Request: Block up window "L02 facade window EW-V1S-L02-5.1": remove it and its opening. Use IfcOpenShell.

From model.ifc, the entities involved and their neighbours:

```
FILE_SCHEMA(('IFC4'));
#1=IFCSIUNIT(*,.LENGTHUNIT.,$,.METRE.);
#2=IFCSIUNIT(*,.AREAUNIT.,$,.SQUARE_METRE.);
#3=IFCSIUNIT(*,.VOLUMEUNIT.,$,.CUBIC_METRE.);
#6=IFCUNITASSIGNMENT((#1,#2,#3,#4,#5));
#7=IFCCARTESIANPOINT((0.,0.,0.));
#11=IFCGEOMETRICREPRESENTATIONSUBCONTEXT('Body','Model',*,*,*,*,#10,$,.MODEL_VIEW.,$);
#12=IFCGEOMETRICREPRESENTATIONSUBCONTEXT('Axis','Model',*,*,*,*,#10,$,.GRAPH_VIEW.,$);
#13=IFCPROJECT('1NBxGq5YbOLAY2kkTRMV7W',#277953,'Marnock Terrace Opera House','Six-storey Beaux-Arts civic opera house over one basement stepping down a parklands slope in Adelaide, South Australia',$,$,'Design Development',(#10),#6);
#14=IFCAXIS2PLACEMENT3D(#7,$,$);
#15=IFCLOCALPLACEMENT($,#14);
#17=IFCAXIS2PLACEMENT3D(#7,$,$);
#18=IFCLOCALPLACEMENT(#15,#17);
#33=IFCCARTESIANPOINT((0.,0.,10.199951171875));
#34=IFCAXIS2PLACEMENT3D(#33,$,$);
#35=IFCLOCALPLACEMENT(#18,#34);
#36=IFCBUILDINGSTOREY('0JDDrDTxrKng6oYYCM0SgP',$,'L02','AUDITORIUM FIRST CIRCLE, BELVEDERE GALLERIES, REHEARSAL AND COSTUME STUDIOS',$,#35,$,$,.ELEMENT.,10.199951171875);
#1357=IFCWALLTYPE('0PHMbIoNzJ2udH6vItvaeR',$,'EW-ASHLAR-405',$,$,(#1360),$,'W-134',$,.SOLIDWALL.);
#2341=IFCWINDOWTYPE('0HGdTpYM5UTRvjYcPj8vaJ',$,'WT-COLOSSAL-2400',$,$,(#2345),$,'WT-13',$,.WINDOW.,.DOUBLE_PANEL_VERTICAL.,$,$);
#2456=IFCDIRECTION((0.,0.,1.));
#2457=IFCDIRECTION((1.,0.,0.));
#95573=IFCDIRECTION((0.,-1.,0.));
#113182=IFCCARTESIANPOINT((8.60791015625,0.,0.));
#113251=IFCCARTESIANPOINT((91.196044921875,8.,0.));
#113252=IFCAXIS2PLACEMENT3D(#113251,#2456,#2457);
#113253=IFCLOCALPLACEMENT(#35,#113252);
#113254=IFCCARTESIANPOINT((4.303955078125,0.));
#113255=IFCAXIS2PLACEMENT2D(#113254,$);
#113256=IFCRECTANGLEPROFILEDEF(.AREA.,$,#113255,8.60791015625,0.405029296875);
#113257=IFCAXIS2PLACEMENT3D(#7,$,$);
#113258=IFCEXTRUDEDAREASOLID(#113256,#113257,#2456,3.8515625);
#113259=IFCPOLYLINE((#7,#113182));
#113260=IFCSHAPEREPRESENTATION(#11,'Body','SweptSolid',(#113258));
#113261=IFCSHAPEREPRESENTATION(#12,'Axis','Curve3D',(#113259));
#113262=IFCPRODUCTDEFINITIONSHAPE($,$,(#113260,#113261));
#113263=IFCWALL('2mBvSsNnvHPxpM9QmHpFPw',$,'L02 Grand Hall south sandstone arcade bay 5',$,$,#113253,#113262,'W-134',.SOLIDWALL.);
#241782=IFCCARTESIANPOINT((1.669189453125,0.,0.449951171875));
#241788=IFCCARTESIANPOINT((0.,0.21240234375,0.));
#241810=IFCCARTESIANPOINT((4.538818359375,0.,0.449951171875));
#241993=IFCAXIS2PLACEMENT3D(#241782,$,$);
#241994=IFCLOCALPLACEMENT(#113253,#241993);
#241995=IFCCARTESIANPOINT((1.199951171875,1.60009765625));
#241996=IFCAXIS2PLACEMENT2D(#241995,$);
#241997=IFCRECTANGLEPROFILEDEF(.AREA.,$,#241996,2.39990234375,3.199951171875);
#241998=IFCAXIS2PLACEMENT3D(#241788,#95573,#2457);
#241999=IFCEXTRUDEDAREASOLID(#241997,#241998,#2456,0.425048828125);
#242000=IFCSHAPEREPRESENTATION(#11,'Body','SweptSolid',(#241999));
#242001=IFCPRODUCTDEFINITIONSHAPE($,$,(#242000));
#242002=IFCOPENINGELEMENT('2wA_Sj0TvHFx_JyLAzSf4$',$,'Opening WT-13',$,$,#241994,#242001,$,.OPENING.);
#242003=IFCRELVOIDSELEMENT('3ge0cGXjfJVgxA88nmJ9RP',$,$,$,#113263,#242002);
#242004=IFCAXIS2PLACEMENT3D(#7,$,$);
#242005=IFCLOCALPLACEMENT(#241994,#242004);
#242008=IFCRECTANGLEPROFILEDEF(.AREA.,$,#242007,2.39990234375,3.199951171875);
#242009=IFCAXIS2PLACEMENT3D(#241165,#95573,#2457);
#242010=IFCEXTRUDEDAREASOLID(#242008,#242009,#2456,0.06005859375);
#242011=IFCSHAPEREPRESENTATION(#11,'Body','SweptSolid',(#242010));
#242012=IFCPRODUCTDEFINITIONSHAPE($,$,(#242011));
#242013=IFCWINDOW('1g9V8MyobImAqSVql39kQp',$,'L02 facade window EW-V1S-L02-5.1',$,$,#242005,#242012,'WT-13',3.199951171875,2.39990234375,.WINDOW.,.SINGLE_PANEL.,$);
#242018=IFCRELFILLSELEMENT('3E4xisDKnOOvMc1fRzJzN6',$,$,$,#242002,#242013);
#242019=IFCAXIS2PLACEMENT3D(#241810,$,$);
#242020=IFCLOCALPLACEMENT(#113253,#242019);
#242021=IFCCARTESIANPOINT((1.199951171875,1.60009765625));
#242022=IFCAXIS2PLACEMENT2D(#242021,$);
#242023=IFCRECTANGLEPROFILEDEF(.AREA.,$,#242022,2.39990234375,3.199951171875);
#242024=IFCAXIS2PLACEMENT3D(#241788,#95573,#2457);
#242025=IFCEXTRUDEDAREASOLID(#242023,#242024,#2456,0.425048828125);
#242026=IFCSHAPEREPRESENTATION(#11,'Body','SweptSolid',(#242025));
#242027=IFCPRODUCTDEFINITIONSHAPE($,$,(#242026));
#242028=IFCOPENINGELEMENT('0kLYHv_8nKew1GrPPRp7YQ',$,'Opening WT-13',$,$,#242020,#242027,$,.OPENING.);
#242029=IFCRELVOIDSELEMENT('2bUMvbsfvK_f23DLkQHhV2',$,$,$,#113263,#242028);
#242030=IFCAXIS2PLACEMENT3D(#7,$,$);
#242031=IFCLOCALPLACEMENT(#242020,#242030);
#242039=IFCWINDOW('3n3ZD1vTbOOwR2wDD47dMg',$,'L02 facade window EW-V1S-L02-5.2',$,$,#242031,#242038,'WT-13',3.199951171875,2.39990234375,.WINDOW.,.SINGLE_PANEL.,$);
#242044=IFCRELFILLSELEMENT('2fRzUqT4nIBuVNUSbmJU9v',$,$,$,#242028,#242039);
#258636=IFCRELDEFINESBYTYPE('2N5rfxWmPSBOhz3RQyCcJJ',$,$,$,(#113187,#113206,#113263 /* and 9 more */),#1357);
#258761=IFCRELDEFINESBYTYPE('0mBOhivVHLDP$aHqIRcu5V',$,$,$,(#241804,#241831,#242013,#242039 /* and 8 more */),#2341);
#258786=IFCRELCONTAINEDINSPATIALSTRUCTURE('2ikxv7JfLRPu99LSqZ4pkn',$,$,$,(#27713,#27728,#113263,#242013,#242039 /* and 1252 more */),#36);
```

```python
import ifcopenshell
import ifcopenshell.api.feature
import ifcopenshell.api.root
import ifcopenshell.geom
import ifcopenshell.util.shape

model = ifcopenshell.open("model.ifc")
settings = ifcopenshell.geom.settings()


def volume(element):
    """Net volume in cubic metres, openings subtracted."""
    shape = ifcopenshell.geom.create_shape(settings, element)
    return ifcopenshell.util.shape.get_volume(shape.geometry)


window = model.by_id(242013)
opening = window.FillsVoids[0].RelatingOpeningElement
wall = opening.VoidsElements[0].RelatingBuildingElement
before = volume(wall)

ifcopenshell.api.root.remove_product(model, product=window)
ifcopenshell.api.feature.remove_feature(model, feature=opening)

after = volume(wall)

print(f"wall volume {before:.3f} -> {after:.3f} m3")

model.write("model-out.ifc")
```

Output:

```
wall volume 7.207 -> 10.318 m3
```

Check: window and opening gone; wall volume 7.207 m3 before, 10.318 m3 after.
